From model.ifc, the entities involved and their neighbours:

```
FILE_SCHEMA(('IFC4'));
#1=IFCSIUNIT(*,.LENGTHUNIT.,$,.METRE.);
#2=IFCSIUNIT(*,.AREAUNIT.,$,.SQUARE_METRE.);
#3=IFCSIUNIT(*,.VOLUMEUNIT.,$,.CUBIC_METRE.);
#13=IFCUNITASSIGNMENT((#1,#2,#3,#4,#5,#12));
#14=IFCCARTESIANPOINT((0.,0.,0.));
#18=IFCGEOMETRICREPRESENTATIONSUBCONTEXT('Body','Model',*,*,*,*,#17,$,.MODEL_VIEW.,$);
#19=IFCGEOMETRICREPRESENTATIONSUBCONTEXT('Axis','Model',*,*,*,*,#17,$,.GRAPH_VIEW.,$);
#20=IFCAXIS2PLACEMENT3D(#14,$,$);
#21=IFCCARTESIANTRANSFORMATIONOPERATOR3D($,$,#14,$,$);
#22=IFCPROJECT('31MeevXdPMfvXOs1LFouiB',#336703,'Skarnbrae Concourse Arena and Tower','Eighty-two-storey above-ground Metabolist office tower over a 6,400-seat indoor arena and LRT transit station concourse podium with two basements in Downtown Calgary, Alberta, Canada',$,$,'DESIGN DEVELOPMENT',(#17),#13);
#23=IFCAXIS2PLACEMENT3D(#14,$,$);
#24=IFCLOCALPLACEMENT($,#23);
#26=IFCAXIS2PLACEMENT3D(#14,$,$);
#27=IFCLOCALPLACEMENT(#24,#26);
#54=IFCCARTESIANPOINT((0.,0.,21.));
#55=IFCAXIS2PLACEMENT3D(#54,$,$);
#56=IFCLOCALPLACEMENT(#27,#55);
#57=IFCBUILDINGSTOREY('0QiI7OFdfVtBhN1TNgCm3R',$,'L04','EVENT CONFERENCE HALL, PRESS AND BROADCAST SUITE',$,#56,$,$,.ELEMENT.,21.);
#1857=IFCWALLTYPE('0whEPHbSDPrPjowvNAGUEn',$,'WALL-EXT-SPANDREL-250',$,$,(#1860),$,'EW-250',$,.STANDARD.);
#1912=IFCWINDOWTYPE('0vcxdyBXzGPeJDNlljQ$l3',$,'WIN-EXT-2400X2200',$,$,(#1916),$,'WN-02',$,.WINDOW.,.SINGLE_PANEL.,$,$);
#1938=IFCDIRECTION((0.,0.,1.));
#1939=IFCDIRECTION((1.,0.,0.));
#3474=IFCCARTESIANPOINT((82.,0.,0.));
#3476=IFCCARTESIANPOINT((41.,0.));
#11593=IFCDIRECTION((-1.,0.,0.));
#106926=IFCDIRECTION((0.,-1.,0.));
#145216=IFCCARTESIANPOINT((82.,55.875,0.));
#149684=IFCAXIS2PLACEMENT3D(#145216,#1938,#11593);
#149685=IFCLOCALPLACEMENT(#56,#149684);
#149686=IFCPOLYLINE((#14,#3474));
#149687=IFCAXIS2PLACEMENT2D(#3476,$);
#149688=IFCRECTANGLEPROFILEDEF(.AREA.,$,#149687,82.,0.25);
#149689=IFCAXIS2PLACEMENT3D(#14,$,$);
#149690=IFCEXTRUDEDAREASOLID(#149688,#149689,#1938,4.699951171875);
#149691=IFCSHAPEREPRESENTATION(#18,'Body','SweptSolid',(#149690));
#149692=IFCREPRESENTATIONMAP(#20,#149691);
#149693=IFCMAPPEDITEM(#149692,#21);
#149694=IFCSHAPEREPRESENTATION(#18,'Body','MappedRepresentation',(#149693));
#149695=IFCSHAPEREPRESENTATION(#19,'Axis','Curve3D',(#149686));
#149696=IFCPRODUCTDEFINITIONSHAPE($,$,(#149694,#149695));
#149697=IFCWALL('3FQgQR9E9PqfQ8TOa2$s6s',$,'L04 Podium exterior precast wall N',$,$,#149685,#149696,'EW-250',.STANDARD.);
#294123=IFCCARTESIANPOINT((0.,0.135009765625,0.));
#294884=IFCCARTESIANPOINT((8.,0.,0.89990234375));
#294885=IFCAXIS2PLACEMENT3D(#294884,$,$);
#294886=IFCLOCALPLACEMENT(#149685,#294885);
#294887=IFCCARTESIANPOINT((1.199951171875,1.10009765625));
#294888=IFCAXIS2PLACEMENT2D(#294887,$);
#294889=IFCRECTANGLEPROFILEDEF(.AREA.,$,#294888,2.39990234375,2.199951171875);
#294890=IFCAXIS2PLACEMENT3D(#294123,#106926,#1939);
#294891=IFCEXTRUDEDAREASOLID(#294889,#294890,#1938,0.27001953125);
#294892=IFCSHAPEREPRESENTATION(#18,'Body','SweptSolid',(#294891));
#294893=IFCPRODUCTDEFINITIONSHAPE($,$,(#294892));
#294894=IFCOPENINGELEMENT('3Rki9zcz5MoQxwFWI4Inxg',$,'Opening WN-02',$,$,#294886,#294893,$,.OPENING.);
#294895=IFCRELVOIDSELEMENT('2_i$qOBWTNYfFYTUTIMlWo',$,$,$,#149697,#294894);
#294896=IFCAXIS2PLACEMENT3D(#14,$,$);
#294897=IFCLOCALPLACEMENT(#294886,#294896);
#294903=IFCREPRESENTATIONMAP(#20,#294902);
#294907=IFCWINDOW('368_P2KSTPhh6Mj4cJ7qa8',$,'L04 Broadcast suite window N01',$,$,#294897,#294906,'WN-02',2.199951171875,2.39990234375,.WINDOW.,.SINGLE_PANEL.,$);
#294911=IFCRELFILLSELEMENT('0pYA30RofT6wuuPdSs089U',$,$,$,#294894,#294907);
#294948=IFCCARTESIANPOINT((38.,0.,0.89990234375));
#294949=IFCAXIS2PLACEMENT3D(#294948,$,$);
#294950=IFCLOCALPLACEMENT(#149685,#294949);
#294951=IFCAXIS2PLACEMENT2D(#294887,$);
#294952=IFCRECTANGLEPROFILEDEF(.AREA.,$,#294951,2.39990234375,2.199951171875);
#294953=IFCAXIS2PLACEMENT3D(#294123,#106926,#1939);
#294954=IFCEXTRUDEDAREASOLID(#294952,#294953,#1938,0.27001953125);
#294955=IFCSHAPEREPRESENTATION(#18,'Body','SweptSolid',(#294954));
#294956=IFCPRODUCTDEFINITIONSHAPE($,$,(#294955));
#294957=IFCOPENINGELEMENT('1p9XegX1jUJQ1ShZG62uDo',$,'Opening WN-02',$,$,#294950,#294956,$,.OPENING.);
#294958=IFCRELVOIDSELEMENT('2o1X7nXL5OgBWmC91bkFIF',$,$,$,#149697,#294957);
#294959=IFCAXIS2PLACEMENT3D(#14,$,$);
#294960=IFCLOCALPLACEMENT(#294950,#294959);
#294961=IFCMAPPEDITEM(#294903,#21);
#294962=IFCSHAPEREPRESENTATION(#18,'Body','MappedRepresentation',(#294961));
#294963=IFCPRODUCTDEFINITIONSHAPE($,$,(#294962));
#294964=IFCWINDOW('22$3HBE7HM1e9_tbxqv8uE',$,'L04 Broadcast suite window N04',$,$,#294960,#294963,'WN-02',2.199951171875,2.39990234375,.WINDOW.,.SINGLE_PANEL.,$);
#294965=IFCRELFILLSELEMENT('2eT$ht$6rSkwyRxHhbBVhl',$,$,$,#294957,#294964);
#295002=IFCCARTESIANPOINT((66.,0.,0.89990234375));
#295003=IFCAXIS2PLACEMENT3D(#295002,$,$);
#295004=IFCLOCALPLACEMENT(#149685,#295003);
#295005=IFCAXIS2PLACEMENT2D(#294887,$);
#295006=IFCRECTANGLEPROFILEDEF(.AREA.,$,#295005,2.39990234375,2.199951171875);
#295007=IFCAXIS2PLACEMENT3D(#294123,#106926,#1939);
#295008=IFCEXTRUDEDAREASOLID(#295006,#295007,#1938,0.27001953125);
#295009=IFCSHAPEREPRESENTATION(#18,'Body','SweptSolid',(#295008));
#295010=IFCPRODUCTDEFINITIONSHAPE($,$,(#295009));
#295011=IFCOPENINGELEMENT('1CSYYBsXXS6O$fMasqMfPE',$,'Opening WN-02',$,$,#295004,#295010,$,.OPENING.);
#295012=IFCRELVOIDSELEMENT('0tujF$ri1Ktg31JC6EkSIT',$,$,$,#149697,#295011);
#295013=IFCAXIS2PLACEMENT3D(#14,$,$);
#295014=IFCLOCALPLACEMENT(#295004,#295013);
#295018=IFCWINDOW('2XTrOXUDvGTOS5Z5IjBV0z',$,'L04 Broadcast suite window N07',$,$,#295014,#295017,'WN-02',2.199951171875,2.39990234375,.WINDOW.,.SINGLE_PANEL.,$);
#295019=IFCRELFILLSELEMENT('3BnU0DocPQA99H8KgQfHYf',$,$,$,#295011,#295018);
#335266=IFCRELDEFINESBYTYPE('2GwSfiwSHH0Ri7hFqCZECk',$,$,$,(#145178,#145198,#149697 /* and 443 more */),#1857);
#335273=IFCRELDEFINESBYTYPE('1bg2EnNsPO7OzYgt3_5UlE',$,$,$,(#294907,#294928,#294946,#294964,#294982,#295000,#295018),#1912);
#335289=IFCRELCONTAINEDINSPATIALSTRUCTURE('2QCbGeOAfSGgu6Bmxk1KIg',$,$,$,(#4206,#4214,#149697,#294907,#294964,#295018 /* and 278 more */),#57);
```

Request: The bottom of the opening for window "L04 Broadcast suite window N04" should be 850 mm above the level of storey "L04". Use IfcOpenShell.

```python
import numpy as np
import ifcopenshell
import ifcopenshell.api.geometry
import ifcopenshell.geom
import ifcopenshell.util.element
import ifcopenshell.util.placement
import ifcopenshell.util.shape
import ifcopenshell.util.unit

model = ifcopenshell.open("model.ifc")
unit_scale = ifcopenshell.util.unit.calculate_unit_scale(model)

window = model.by_guid("22$3HBE7HM1e9_tbxqv8uE")
opening = window.FillsVoids[0].RelatingOpeningElement
storey = ifcopenshell.util.element.get_container(window, ifc_class="IfcBuildingStorey")
level = ifcopenshell.util.placement.get_local_placement(storey.ObjectPlacement)[2, 3]

# The opening's origin need not be at the sill, so measure its lowest point.
shape = ifcopenshell.geom.create_shape(ifcopenshell.geom.settings(), opening)
bottom = ifcopenshell.util.shape.get_shape_bottom_elevation(shape, shape.geometry) / unit_scale
dz = level + 0.85 / unit_scale - bottom

shift = np.array([0.0, 0.0, dz])
# The window is placed relative to its opening, so it follows when the opening moves.
matrix = ifcopenshell.util.placement.get_local_placement(opening.ObjectPlacement)
matrix[:3, 3] += shift
ifcopenshell.api.geometry.edit_object_placement(
    model, product=opening, matrix=matrix, is_si=False, should_transform_children=True
)

print(f"moved by {dz * unit_scale:+.3f} m")

model.write("model_edited.ifc")
```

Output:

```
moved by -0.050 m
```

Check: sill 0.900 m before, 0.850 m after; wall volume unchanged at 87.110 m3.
